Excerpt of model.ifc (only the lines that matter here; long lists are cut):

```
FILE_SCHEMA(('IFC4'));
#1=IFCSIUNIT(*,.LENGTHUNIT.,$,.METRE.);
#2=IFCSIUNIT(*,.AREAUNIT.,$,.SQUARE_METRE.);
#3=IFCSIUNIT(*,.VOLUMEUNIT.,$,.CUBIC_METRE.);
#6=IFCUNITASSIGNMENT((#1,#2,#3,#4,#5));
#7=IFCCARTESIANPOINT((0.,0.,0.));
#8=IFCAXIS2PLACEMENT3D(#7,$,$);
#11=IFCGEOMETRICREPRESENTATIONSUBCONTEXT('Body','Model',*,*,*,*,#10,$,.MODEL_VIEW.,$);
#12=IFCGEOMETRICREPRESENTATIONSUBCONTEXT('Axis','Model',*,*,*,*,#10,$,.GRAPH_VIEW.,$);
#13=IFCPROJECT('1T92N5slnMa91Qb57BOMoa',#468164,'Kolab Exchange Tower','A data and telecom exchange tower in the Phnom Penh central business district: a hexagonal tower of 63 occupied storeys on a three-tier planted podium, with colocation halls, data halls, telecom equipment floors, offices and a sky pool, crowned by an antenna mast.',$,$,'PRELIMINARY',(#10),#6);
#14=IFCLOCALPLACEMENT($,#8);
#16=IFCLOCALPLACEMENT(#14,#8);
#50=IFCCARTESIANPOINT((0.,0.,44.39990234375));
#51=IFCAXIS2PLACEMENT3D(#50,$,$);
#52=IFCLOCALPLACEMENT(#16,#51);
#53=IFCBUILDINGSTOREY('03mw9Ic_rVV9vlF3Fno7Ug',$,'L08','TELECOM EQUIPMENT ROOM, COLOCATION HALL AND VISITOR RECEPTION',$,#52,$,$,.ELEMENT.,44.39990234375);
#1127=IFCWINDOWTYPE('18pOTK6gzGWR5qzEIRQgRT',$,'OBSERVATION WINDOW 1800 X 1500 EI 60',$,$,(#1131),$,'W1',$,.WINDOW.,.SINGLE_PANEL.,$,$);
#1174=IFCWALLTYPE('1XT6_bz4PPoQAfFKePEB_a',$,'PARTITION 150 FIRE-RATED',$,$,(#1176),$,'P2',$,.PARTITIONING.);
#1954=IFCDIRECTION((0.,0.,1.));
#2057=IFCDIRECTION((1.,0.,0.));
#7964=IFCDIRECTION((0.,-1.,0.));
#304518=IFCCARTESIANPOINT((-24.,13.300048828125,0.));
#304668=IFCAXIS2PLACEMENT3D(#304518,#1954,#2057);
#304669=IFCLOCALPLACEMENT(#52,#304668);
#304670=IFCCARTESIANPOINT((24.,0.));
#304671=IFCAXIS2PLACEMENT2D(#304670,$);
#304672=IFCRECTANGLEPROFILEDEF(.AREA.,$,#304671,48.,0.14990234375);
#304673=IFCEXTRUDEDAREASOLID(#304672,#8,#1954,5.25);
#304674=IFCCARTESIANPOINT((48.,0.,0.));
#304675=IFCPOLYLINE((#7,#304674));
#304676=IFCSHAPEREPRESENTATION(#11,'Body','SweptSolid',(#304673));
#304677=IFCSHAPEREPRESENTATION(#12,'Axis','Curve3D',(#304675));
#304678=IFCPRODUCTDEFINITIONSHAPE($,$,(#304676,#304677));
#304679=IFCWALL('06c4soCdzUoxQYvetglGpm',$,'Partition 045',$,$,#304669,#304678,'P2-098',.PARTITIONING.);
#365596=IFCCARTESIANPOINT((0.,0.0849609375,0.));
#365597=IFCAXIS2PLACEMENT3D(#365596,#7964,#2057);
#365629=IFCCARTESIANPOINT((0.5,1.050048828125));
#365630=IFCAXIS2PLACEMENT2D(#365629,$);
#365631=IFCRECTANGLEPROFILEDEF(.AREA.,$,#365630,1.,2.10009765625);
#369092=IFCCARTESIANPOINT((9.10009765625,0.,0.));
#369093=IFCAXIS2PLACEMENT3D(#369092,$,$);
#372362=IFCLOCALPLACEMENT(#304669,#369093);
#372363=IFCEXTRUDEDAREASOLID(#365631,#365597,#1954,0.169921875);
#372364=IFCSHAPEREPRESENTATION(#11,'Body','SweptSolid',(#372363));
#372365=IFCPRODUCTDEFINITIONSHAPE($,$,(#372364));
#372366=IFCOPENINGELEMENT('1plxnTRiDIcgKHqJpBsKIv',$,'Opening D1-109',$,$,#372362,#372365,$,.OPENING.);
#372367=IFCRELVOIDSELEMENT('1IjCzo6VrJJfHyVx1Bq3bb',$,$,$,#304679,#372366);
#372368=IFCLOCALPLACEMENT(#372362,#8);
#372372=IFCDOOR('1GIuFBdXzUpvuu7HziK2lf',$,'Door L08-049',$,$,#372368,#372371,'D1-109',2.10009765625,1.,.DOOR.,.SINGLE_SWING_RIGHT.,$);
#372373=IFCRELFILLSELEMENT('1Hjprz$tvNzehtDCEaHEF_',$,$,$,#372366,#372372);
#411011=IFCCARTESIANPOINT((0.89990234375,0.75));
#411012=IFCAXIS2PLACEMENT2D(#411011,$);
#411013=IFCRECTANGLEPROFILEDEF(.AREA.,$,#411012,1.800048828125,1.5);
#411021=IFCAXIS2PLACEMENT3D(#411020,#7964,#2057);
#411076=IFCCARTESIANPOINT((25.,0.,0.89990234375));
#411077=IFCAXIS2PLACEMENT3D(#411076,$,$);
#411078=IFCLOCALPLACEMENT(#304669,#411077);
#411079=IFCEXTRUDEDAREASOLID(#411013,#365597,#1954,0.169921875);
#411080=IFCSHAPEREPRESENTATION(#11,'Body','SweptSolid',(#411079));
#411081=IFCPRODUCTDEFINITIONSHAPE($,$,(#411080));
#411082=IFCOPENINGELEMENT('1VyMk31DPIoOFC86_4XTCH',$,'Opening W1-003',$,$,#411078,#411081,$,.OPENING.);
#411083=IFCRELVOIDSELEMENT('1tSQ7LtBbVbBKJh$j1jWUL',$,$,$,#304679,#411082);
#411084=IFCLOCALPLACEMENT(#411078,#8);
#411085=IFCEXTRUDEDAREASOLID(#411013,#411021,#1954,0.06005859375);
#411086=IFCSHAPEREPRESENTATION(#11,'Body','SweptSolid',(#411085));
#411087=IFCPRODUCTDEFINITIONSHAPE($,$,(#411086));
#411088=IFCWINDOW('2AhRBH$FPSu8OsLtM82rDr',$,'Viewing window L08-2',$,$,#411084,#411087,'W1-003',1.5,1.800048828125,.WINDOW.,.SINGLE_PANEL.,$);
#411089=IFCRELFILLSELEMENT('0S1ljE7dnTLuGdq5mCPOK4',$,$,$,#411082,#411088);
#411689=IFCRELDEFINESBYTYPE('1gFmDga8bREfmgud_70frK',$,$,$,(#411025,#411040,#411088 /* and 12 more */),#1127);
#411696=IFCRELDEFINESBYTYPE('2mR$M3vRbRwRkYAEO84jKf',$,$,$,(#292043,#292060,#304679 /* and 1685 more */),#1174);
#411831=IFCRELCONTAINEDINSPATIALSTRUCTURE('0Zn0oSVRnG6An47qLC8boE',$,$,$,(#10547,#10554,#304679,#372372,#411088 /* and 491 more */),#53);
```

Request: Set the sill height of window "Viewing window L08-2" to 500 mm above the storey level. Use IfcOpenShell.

```python
import numpy as np
import ifcopenshell
import ifcopenshell.api.geometry
import ifcopenshell.geom
import ifcopenshell.util.element
import ifcopenshell.util.placement
import ifcopenshell.util.shape
import ifcopenshell.util.unit

model = ifcopenshell.open("model.ifc")
unit_scale = ifcopenshell.util.unit.calculate_unit_scale(model)

window = model.by_guid("2AhRBH$FPSu8OsLtM82rDr")
opening = window.FillsVoids[0].RelatingOpeningElement
storey = ifcopenshell.util.element.get_container(window, ifc_class="IfcBuildingStorey")
level = ifcopenshell.util.placement.get_local_placement(storey.ObjectPlacement)[2, 3]

# The opening's origin need not be at the sill, so measure its lowest point.
shape = ifcopenshell.geom.create_shape(ifcopenshell.geom.settings(), opening)
bottom = ifcopenshell.util.shape.get_shape_bottom_elevation(shape, shape.geometry) / unit_scale
dz = level + 0.5 / unit_scale - bottom

shift = np.array([0.0, 0.0, dz])
# The window is placed relative to its opening, so it follows when the opening moves.
matrix = ifcopenshell.util.placement.get_local_placement(opening.ObjectPlacement)
matrix[:3, 3] += shift
ifcopenshell.api.geometry.edit_object_placement(
    model, product=opening, matrix=matrix, is_si=False, should_transform_children=True
)

print(f"moved by {dz * unit_scale:+.3f} m")

model.write("model-out.ifc")
```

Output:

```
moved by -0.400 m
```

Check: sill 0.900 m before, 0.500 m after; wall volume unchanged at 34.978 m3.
